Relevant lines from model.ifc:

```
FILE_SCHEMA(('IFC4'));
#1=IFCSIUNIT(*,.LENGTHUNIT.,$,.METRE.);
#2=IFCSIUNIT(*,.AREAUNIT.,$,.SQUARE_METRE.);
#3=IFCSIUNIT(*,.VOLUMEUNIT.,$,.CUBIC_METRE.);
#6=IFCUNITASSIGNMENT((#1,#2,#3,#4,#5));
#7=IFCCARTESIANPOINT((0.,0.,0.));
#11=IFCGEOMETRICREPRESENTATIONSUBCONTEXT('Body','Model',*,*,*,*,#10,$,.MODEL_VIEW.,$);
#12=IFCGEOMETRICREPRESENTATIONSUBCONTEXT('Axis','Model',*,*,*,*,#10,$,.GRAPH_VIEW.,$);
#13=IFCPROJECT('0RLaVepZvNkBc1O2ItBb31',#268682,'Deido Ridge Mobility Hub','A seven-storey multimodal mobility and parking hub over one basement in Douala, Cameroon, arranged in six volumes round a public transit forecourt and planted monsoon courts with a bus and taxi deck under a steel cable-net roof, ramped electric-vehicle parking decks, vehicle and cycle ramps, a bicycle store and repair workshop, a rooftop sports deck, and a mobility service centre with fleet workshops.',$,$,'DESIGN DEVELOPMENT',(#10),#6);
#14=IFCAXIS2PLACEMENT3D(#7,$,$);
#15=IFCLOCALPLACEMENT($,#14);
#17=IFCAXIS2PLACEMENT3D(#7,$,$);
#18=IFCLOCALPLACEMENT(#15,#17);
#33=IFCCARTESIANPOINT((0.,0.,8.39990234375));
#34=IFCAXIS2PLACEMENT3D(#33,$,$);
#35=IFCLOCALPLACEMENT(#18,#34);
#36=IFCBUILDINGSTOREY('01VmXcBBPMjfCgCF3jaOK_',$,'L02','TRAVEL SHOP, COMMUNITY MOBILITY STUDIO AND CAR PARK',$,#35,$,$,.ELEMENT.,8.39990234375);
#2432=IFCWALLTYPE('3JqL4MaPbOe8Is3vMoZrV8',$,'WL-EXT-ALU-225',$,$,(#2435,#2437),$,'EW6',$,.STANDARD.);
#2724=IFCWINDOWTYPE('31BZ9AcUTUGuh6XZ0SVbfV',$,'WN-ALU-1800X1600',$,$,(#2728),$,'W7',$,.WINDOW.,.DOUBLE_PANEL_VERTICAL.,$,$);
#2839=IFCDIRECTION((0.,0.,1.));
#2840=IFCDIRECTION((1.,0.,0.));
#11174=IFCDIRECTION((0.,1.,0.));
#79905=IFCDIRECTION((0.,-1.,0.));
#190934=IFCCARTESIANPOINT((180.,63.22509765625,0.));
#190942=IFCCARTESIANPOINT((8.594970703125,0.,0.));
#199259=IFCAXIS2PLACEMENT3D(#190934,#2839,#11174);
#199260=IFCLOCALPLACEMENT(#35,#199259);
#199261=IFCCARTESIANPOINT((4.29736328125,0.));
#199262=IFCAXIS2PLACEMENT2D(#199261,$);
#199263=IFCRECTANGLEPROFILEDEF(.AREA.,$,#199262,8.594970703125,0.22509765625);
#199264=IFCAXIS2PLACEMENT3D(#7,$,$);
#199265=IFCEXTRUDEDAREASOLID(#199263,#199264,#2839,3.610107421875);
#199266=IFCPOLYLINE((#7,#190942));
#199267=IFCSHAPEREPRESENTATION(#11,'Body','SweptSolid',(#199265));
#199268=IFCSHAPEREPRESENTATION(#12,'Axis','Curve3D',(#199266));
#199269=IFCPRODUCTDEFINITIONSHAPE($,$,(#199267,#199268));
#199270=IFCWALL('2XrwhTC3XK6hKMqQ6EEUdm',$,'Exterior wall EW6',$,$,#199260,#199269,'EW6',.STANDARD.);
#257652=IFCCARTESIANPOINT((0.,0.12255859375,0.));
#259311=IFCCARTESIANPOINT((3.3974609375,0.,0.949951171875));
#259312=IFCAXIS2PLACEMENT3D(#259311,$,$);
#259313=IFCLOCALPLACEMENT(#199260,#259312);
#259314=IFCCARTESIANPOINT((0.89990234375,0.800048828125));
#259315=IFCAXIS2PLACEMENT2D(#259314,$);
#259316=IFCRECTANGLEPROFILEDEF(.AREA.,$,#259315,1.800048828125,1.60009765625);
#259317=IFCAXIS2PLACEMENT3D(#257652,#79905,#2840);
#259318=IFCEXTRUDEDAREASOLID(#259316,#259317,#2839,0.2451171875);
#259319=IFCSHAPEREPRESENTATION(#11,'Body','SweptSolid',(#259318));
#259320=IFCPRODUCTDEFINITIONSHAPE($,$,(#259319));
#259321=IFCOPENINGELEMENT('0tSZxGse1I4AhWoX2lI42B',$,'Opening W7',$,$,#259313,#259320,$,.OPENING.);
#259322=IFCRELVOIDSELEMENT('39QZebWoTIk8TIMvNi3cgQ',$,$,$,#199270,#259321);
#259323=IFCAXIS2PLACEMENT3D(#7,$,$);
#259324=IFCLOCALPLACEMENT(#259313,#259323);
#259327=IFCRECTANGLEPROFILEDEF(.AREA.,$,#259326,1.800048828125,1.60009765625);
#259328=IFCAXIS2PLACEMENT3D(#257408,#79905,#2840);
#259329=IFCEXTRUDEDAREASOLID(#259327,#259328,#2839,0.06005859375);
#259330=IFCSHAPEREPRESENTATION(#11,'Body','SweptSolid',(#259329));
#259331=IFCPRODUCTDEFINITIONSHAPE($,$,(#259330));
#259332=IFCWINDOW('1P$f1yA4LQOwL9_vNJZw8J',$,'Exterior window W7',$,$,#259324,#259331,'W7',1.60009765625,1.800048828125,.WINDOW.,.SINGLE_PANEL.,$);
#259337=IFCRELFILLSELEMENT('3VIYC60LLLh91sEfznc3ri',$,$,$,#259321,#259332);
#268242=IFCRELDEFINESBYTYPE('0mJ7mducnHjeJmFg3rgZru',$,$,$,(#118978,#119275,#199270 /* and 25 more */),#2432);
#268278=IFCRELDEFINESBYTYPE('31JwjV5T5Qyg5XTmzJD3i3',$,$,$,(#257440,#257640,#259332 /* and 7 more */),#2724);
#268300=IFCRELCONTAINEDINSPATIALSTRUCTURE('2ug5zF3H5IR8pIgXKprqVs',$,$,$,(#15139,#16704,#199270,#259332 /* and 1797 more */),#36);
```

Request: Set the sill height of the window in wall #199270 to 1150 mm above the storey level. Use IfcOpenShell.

```python
import numpy as np
import ifcopenshell
import ifcopenshell.api.geometry
import ifcopenshell.geom
import ifcopenshell.util.element
import ifcopenshell.util.placement
import ifcopenshell.util.shape
import ifcopenshell.util.unit

model = ifcopenshell.open("model.ifc")
unit_scale = ifcopenshell.util.unit.calculate_unit_scale(model)

window = model.by_guid("1P$f1yA4LQOwL9_vNJZw8J")
opening = window.FillsVoids[0].RelatingOpeningElement
storey = ifcopenshell.util.element.get_container(window, ifc_class="IfcBuildingStorey")
level = ifcopenshell.util.placement.get_local_placement(storey.ObjectPlacement)[2, 3]

# The opening's origin need not be at the sill, so measure its lowest point.
shape = ifcopenshell.geom.create_shape(ifcopenshell.geom.settings(), opening)
bottom = ifcopenshell.util.shape.get_shape_bottom_elevation(shape, shape.geometry) / unit_scale
dz = level + 1.15 / unit_scale - bottom

shift = np.array([0.0, 0.0, dz])
# The window is placed relative to its opening, so it follows when the opening moves.
matrix = ifcopenshell.util.placement.get_local_placement(opening.ObjectPlacement)
matrix[:3, 3] += shift
ifcopenshell.api.geometry.edit_object_placement(
    model, product=opening, matrix=matrix, is_si=False, should_transform_children=True
)

print(f"moved by {dz * unit_scale:+.3f} m")

model.write("model_updated.ifc")
```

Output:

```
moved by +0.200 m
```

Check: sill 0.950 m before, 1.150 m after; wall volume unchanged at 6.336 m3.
